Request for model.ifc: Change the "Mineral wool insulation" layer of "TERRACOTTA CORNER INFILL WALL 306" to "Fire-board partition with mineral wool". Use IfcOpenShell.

First a look at what the model holds.

```python
import ifcopenshell
import ifcopenshell.util.element

model = ifcopenshell.open("model.ifc")
print(model.schema)
for layer_set in model.by_type("IfcMaterialLayerSet"):
    if layer_set.LayerSetName == "TERRACOTTA CORNER INFILL WALL 306":
        for layer in layer_set.MaterialLayers:
            print(layer.id(), layer.Material and layer.Material.Name, layer.LayerThickness, sep=" | ")
        print(len(ifcopenshell.util.element.get_elements_by_material(model, layer_set)), "elements and types use it")
print(sorted(m.Name for m in model.by_type("IfcMaterial") if m.Name)[:60])
```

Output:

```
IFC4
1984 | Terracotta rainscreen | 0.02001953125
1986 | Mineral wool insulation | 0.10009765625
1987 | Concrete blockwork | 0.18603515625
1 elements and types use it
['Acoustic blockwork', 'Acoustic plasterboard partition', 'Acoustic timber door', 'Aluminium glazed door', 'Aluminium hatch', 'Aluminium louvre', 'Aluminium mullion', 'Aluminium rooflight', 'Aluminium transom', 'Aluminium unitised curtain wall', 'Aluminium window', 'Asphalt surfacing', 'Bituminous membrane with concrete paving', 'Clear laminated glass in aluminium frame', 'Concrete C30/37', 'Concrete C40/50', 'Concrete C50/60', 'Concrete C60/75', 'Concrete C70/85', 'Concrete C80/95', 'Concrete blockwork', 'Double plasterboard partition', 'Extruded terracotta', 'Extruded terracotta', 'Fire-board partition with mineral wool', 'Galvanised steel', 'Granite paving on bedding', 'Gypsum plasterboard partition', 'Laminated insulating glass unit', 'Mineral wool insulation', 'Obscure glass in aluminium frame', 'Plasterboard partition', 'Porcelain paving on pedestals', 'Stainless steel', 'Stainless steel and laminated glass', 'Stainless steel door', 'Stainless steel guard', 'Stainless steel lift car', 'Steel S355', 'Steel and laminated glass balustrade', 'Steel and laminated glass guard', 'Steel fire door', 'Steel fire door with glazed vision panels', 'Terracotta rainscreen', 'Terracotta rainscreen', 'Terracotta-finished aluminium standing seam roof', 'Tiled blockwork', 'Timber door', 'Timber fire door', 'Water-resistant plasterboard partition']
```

```python
import ifcopenshell
import ifcopenshell.api.material

model = ifcopenshell.open("model.ifc")

layer_set = next(s for s in model.by_type("IfcMaterialLayerSet") if s.LayerSetName == "TERRACOTTA CORNER INFILL WALL 306")
layer = next(l for l in layer_set.MaterialLayers if l.Material and l.Material.Name == "Mineral wool insulation")
material = next(m for m in model.by_type("IfcMaterial") if m.Name == "Fire-board partition with mineral wool")

# Point this one layer at the other material; renaming the old one would change it everywhere.
ifcopenshell.api.material.edit_layer(model, layer=layer, attributes={}, material=material)

print([l.Material.Name if l.Material else None for l in layer_set.MaterialLayers])

model.write("model_edited.ifc")
```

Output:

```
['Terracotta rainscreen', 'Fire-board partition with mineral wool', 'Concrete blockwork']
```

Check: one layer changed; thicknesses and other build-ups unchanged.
